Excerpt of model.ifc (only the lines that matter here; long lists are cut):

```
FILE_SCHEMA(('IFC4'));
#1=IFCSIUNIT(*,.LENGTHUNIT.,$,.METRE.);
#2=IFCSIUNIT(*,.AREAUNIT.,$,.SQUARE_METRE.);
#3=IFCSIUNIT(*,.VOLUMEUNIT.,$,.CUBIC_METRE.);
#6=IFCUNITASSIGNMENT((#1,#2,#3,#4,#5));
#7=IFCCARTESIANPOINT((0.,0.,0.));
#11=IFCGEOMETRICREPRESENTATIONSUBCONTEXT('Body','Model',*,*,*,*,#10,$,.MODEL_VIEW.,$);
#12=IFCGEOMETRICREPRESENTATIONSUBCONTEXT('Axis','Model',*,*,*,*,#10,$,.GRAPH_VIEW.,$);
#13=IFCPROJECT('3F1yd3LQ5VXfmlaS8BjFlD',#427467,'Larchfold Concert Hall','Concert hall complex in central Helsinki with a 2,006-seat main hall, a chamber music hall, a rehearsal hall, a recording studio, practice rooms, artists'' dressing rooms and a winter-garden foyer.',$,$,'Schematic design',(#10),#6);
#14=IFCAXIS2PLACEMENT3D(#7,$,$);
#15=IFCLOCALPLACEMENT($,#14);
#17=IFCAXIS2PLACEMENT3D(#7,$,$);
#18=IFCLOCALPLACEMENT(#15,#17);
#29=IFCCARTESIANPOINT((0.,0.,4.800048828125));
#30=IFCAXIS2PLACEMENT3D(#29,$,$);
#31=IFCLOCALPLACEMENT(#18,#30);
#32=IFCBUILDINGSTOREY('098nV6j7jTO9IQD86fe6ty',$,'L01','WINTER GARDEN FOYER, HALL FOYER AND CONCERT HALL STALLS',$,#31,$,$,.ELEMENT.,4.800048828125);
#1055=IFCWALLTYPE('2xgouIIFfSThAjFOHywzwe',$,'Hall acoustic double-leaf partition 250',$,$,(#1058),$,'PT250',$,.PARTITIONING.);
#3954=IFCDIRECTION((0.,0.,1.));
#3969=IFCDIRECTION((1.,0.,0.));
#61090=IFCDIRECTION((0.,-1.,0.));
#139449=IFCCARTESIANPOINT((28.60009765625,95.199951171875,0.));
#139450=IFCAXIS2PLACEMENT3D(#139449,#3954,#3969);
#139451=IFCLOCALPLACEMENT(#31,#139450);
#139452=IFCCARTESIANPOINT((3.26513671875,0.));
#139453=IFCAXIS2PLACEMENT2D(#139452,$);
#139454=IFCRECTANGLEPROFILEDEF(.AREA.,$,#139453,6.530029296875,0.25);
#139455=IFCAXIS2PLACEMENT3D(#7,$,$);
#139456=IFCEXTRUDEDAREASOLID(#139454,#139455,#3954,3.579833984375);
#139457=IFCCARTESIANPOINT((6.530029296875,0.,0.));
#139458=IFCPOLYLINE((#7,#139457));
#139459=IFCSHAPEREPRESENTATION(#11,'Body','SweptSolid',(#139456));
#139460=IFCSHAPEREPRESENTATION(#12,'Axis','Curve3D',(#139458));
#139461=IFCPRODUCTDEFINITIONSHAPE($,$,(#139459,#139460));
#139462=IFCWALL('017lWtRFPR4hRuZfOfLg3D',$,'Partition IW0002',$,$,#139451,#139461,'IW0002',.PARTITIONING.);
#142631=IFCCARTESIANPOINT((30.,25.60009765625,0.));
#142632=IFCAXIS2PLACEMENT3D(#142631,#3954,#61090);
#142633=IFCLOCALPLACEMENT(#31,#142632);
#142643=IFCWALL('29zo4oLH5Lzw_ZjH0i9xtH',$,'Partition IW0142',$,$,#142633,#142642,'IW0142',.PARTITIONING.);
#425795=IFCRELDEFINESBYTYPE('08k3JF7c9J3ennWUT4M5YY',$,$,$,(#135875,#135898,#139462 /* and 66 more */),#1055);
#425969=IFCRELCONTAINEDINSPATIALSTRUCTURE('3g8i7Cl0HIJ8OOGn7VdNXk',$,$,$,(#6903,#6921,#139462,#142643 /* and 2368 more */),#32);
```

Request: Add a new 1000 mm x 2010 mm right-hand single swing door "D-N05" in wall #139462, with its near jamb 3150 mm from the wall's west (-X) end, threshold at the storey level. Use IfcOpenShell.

```python
import numpy as np
import ifcopenshell
import ifcopenshell.api.feature
import ifcopenshell.api.geometry
import ifcopenshell.api.root
import ifcopenshell.api.spatial
import ifcopenshell.geom
import ifcopenshell.util.element
import ifcopenshell.util.placement
import ifcopenshell.util.representation
import ifcopenshell.util.shape
import ifcopenshell.util.unit

model = ifcopenshell.open("model.ifc")
unit_scale = ifcopenshell.util.unit.calculate_unit_scale(model)
settings = ifcopenshell.geom.settings()


def volume(element):
    """Net volume in cubic metres, openings subtracted."""
    shape = ifcopenshell.geom.create_shape(settings, element)
    return ifcopenshell.util.shape.get_volume(shape.geometry)


wall = model.by_guid("017lWtRFPR4hRuZfOfLg3D")
storey = ifcopenshell.util.element.get_container(wall, ifc_class="IfcBuildingStorey")
context = ifcopenshell.util.representation.get_context(model, "Model", "Body", "MODEL_VIEW")
before = volume(wall)

width, height, from_end, sill = 1, 2.01, 3.15, 0.0  # metres

# The wall runs along its own X axis, and the end named is its -X end.
wall_shape = ifcopenshell.geom.create_shape(settings, wall)
x, y, z = ifcopenshell.util.shape.get_vertices(wall_shape.geometry).T
start = x.min() + from_end
face, thickness = float(y.min()), float(y.max() - y.min())
wall_matrix = ifcopenshell.util.placement.get_local_placement(wall.ObjectPlacement)
level = ifcopenshell.util.placement.get_local_placement(storey.ObjectPlacement)[2, 3]


def in_wall(x, y):
    """Placement at x, y metres in the wall's axes, at sill height."""
    matrix = wall_matrix.copy()
    matrix[:, 3] = wall_matrix @ np.array([x / unit_scale, y / unit_scale, 0.0, 1.0])
    matrix[2, 3] = level + sill / unit_scale
    return matrix


# Opening: a box that overshoots both wall faces by 50 mm.
opening = ifcopenshell.api.root.create_entity(model, ifc_class="IfcOpeningElement", predefined_type="OPENING")
box = ifcopenshell.api.geometry.add_wall_representation(
    model, context=context, length=width, height=height, thickness=thickness + 0.1
)
ifcopenshell.api.geometry.assign_representation(model, product=opening, representation=box)
ifcopenshell.api.geometry.edit_object_placement(model, product=opening, matrix=in_wall(start, face - 0.05), is_si=False)
ifcopenshell.api.feature.add_feature(model, feature=opening, element=wall)

door = ifcopenshell.api.root.create_entity(model, ifc_class="IfcDoor", name="D-N05", predefined_type="DOOR")
door.OverallWidth, door.OverallHeight = width / unit_scale, height / unit_scale
door.OperationType = "SINGLE_SWING_RIGHT"
body = ifcopenshell.api.geometry.add_door_representation(
    model,
    context=context,
    overall_width=door.OverallWidth,
    overall_height=door.OverallHeight,
    operation_type="SINGLE_SWING_RIGHT",
    lining_properties={"LiningDepth": thickness / unit_scale, "ThresholdDepth": thickness / unit_scale},
)
ifcopenshell.api.geometry.assign_representation(model, product=door, representation=body)
ifcopenshell.api.spatial.assign_container(model, products=[door], relating_structure=storey)
ifcopenshell.api.feature.add_filling(model, opening=opening, element=door)

# The lining spans the wall, so the door starts at the wall face.
ifcopenshell.api.geometry.edit_object_placement(model, product=door, matrix=in_wall(start, face), is_si=False)

after = volume(wall)

print(f"wall volume {before:.3f} -> {after:.3f} m3")

model.write("model_rev.ifc")
```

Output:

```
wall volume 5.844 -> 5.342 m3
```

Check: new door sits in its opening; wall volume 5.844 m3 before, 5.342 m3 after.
